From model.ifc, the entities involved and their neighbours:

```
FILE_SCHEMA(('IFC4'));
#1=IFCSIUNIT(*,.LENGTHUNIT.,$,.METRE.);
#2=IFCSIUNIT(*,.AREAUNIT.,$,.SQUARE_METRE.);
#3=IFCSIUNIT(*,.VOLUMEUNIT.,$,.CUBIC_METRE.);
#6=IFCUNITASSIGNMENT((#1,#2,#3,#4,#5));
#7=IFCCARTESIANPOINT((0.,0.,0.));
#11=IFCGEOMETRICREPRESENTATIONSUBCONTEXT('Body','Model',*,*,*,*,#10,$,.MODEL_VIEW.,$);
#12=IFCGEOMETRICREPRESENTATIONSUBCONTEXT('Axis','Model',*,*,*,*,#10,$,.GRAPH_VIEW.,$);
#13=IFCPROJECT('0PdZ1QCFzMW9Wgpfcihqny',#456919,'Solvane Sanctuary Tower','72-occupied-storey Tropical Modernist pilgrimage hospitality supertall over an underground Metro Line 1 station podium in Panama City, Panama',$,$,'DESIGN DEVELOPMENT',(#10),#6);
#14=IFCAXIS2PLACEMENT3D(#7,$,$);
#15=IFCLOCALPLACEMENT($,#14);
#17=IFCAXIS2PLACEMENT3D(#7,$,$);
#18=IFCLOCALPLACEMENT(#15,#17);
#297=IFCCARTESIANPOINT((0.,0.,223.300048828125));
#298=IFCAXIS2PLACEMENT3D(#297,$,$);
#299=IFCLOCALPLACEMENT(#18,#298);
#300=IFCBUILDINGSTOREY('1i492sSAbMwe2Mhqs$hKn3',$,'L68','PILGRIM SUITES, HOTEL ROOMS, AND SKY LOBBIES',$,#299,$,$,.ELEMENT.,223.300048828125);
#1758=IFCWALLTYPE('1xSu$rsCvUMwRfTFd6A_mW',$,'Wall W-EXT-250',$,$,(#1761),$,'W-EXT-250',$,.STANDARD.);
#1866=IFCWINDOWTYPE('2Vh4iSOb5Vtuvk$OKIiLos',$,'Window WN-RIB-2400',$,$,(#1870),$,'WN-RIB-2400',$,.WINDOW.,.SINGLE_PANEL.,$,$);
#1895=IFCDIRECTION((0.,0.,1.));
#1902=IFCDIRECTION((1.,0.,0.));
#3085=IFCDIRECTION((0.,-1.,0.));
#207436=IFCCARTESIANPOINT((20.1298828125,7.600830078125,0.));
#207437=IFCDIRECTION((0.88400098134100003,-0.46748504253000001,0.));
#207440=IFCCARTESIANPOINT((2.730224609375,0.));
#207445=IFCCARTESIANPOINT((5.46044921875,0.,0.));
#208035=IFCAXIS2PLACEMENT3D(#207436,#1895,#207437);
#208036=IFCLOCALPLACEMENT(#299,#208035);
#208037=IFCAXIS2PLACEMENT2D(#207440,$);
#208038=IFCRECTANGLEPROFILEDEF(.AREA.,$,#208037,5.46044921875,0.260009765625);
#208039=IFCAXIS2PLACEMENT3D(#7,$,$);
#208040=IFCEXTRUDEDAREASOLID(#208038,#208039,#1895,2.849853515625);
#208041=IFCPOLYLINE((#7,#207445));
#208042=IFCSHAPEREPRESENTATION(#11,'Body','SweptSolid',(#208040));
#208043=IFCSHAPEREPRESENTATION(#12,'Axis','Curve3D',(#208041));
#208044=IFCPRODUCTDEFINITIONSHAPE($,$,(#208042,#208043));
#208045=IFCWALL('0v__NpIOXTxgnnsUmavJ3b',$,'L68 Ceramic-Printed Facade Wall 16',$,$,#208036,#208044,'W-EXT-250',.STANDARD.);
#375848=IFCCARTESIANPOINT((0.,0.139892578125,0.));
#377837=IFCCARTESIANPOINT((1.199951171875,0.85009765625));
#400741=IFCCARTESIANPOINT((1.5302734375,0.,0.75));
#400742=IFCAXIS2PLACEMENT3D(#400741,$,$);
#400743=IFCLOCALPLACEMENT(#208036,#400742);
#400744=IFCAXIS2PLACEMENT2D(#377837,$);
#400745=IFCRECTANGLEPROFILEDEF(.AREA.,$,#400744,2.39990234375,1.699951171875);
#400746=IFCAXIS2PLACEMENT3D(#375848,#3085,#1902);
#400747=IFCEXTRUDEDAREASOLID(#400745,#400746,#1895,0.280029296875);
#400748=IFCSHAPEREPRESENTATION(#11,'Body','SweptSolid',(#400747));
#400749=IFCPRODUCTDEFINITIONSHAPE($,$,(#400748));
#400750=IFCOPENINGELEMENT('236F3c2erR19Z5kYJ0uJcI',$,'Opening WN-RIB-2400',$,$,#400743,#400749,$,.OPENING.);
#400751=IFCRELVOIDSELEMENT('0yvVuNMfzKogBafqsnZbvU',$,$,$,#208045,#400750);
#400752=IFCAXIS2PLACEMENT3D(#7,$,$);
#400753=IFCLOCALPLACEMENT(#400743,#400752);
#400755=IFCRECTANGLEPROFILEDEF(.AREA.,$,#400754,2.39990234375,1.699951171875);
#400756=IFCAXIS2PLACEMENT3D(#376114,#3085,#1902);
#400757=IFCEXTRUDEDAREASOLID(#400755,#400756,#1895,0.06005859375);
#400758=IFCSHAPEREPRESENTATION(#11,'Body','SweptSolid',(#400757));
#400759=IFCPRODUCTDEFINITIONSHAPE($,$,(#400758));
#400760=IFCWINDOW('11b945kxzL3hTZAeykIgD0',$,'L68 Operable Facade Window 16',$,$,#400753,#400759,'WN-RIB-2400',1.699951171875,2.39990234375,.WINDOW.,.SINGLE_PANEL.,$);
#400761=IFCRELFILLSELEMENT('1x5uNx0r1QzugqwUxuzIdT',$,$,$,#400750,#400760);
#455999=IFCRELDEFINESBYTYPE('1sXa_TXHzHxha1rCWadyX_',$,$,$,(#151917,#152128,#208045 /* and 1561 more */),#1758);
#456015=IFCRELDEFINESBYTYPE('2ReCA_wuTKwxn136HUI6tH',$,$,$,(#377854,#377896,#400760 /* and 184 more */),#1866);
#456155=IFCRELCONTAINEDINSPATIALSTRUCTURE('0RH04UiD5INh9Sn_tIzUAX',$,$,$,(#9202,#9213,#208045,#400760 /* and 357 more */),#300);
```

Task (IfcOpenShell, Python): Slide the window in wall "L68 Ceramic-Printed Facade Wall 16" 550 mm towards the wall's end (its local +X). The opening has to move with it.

```python
import ifcopenshell
import ifcopenshell.api.geometry
import ifcopenshell.util.placement
import ifcopenshell.util.unit

model = ifcopenshell.open("model.ifc")
unit_scale = ifcopenshell.util.unit.calculate_unit_scale(model)

window = model.by_guid("11b945kxzL3hTZAeykIgD0")
opening = window.FillsVoids[0].RelatingOpeningElement
wall = opening.VoidsElements[0].RelatingBuildingElement

wall_matrix = ifcopenshell.util.placement.get_local_placement(wall.ObjectPlacement)
shift = wall_matrix[:3, 0] * 0.55 / unit_scale
before = ifcopenshell.util.placement.get_local_placement(window.ObjectPlacement)[:3, 3].copy()

# The window is placed relative to its opening, so it follows when the opening moves.
matrix = ifcopenshell.util.placement.get_local_placement(opening.ObjectPlacement)
matrix[:3, 3] += shift
ifcopenshell.api.geometry.edit_object_placement(
    model, product=opening, matrix=matrix, is_si=False, should_transform_children=True
)

after = ifcopenshell.util.placement.get_local_placement(window.ObjectPlacement)[:3, 3]
print("window moved by", (after - before).round(3) + 0.0)

model.write("model_v2.ifc")
```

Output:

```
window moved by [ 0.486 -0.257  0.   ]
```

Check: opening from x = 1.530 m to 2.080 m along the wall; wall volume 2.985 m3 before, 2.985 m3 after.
